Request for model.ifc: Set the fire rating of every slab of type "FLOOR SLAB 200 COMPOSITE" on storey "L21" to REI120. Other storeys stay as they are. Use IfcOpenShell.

First a look at what the model holds.

```python
import ifcopenshell
import ifcopenshell.util.element

model = ifcopenshell.open("model.ifc")
print(model.schema)
storey = next(s for s in model.by_type("IfcBuildingStorey") if s.Name == "L21")
slabs = [e for e in ifcopenshell.util.element.get_decomposition(storey) if e.is_a("IfcSlab")]
seen = {}
for e in slabs:
    element_type = ifcopenshell.util.element.get_type(e)
    key = (element_type.Name if element_type != e and element_type else None, ifcopenshell.util.element.get_pset(e, "Pset_SlabCommon", "FireRating"))
    seen[key] = seen.get(key, 0) + 1
for (name, value), count in sorted(seen.items(), key=str):
    print(count, "x", name, "|", value)
```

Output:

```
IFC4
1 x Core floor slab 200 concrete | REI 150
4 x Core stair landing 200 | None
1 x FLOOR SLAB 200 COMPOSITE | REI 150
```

```python
import ifcopenshell
import ifcopenshell.api.pset
import ifcopenshell.util.element

model = ifcopenshell.open("model.ifc")

storey = next(s for s in model.by_type("IfcBuildingStorey") if s.Name == "L21")
slabs = [e for e in ifcopenshell.util.element.get_decomposition(storey) if e.is_a("IfcSlab")]

count = 0
for e in slabs:
    element_type = ifcopenshell.util.element.get_type(e)
    if element_type in (None, e) or element_type.Name != "FLOOR SLAB 200 COMPOSITE":
        continue
    found = ifcopenshell.util.element.get_pset(e, "Pset_SlabCommon", should_inherit=False)
    if found:
        pset = model.by_id(found["id"])
        if len(ifcopenshell.util.element.get_elements_by_pset(pset)) > 1:
            pset = ifcopenshell.api.pset.unshare_pset(model, products=[e], pset=pset)[0]
    else:
        pset = ifcopenshell.api.pset.add_pset(model, product=e, name="Pset_SlabCommon")
    ifcopenshell.api.pset.edit_pset(model, pset=pset, properties={"FireRating": "REI120"})
    count += 1

print(count, "slabs updated")

model.write("model_rev.ifc")
```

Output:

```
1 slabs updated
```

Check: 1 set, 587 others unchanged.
